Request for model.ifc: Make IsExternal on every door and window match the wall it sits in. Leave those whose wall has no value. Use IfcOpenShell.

First a look at what the model holds.

```python
import ifcopenshell
import ifcopenshell.util.element

model = ifcopenshell.open("model.ifc")
print(model.schema)
seen = {}
for e in model.by_type("IfcDoor") + model.by_type("IfcWindow"):
    if not e.FillsVoids:
        continue
    host = e.FillsVoids[0].RelatingOpeningElement.VoidsElements[0].RelatingBuildingElement
    own = ifcopenshell.util.element.get_pset(e, f"Pset_{e.is_a()[3:].removesuffix('StandardCase')}Common", "IsExternal")
    wall = ifcopenshell.util.element.get_pset(host, "Pset_WallCommon", "IsExternal")
    seen[e.is_a(), own, wall] = seen.get((e.is_a(), own, wall), 0) + 1
for (cls, own, wall), count in sorted(seen.items(), key=str):
    print(count, cls, "IsExternal:", own, "| host wall:", wall)
```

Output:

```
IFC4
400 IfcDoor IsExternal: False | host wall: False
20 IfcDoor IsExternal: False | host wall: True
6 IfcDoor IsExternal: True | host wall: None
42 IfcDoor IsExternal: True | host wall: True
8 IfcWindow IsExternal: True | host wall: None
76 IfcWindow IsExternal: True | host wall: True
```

```python
import ifcopenshell
import ifcopenshell.api.pset
import ifcopenshell.util.element

model = ifcopenshell.open("model.ifc")

count = 0
for ifc_class, pset_name in (("IfcDoor", "Pset_DoorCommon"), ("IfcWindow", "Pset_WindowCommon")):
    for e in model.by_type(ifc_class):
        if not e.FillsVoids:
            continue
        host = e.FillsVoids[0].RelatingOpeningElement.VoidsElements[0].RelatingBuildingElement
        external = ifcopenshell.util.element.get_pset(host, "Pset_WallCommon", "IsExternal")
        if external is None or ifcopenshell.util.element.get_pset(e, pset_name, "IsExternal") == external:
            continue
        pset = ifcopenshell.api.pset.add_pset(model, product=e, name=pset_name)
        ifcopenshell.api.pset.edit_pset(model, pset=pset, properties={"IsExternal": external})
        count += 1

print(count, "updated")

model.write("model_updated.ifc")
```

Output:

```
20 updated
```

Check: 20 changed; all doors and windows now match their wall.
